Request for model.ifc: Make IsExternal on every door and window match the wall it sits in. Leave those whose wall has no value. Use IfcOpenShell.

First a look at what the model holds.

```python
import ifcopenshell
import ifcopenshell.util.element

model = ifcopenshell.open("model.ifc")
print(model.schema)
seen = {}
for e in model.by_type("IfcDoor") + model.by_type("IfcWindow"):
    if not e.FillsVoids:
        continue
    host = e.FillsVoids[0].RelatingOpeningElement.VoidsElements[0].RelatingBuildingElement
    own = ifcopenshell.util.element.get_pset(e, f"Pset_{e.is_a()[3:].removesuffix('StandardCase')}Common", "IsExternal")
    wall = ifcopenshell.util.element.get_pset(host, "Pset_WallCommon", "IsExternal")
    seen[e.is_a(), own, wall] = seen.get((e.is_a(), own, wall), 0) + 1
for (cls, own, wall), count in sorted(seen.items(), key=str):
    print(count, cls, "IsExternal:", own, "| host wall:", wall)
```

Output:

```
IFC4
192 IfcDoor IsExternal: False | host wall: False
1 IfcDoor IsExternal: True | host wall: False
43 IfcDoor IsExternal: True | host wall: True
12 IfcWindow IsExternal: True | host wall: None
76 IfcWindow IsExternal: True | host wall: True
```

```python
import ifcopenshell
import ifcopenshell.api.pset
import ifcopenshell.util.element

model = ifcopenshell.open("model.ifc")

count = 0
for ifc_class, pset_name in (("IfcDoor", "Pset_DoorCommon"), ("IfcWindow", "Pset_WindowCommon")):
    for e in model.by_type(ifc_class):
        if not e.FillsVoids:
            continue
        host = e.FillsVoids[0].RelatingOpeningElement.VoidsElements[0].RelatingBuildingElement
        external = ifcopenshell.util.element.get_pset(host, "Pset_WallCommon", "IsExternal")
        if external is None or ifcopenshell.util.element.get_pset(e, pset_name, "IsExternal") == external:
            continue
        pset = ifcopenshell.api.pset.add_pset(model, product=e, name=pset_name)
        ifcopenshell.api.pset.edit_pset(model, pset=pset, properties={"IsExternal": external})
        count += 1

print(count, "updated")

model.write("model_rev.ifc")
```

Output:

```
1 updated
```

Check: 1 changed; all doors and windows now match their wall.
